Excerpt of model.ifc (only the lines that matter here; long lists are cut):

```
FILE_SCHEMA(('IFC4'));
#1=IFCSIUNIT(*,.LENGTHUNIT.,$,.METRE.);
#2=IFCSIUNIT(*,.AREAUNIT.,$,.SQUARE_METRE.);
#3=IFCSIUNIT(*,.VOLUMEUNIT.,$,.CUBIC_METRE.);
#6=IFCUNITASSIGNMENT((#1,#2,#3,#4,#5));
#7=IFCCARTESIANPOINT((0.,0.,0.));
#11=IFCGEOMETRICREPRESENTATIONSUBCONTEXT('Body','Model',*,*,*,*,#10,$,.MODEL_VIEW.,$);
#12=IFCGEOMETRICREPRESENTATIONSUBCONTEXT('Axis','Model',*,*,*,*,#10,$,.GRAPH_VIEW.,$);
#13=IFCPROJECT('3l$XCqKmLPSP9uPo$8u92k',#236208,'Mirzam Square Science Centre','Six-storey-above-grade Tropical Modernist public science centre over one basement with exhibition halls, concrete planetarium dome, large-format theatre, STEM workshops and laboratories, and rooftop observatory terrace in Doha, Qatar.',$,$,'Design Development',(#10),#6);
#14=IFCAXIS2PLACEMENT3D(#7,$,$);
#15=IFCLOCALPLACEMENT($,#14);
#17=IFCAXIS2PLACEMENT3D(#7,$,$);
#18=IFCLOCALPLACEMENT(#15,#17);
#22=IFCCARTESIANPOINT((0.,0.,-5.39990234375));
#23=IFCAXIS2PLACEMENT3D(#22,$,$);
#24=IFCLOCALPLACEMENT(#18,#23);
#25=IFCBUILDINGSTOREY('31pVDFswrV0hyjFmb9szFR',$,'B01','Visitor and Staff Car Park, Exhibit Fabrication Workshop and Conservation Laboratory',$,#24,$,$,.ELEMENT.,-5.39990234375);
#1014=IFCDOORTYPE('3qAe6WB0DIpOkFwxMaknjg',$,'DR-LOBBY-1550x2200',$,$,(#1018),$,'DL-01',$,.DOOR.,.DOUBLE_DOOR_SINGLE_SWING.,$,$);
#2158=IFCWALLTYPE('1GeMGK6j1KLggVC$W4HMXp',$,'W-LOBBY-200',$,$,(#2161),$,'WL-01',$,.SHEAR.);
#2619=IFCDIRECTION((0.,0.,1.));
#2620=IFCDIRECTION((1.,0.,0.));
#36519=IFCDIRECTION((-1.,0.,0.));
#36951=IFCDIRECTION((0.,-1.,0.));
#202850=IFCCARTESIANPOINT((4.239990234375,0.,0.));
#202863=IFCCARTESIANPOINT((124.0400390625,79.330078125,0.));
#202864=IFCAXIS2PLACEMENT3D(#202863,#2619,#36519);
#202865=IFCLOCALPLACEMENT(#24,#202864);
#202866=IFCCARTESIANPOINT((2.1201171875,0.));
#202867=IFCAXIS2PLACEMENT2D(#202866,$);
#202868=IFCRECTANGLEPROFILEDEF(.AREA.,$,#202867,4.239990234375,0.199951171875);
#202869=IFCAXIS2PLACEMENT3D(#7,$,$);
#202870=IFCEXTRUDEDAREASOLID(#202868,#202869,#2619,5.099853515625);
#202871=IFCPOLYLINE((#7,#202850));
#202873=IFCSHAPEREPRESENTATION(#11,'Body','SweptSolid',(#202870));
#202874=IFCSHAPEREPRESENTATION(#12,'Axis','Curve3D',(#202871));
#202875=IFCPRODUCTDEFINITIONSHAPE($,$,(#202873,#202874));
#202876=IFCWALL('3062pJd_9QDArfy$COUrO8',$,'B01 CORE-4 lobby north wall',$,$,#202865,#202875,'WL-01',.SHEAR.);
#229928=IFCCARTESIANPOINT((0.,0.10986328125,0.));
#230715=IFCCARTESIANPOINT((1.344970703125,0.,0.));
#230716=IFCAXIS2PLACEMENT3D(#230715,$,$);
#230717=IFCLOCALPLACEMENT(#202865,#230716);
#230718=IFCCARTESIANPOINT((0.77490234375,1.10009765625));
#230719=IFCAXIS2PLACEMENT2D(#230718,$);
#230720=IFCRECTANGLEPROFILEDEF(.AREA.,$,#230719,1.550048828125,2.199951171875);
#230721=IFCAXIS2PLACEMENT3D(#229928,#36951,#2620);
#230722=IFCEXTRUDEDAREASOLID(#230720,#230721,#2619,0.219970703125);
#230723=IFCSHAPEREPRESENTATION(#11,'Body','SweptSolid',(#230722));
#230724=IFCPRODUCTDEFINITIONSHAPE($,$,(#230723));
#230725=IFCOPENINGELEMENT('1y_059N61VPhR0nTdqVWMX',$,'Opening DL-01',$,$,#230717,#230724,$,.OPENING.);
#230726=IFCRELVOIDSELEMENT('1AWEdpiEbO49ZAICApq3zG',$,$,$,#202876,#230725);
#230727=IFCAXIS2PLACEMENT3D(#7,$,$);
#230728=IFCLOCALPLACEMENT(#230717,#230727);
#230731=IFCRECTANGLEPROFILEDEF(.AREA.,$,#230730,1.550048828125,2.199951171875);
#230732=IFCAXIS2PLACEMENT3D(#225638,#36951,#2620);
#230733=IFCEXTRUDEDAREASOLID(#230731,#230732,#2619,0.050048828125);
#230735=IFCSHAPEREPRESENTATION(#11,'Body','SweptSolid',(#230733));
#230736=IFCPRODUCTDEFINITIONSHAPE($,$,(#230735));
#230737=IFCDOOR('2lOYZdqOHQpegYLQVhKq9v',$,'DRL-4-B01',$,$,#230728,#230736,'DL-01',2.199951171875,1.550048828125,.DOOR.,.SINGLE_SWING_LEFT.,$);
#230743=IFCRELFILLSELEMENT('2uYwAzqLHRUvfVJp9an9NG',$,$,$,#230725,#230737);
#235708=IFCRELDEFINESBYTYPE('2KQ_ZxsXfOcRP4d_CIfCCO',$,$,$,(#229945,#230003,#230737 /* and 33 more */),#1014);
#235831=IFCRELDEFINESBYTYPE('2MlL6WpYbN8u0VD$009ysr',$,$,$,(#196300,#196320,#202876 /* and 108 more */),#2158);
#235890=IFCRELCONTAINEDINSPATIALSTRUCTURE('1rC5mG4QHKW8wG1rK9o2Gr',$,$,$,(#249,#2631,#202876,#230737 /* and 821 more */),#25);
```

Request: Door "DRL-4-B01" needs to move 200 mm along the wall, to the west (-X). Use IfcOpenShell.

```python
import ifcopenshell
import ifcopenshell.api.geometry
import ifcopenshell.util.placement
import ifcopenshell.util.unit

model = ifcopenshell.open("model.ifc")
unit_scale = ifcopenshell.util.unit.calculate_unit_scale(model)

door = model.by_id(230737)
opening = door.FillsVoids[0].RelatingOpeningElement
wall = opening.VoidsElements[0].RelatingBuildingElement

wall_matrix = ifcopenshell.util.placement.get_local_placement(wall.ObjectPlacement)
shift = wall_matrix[:3, 0] * 0.2 / unit_scale
before = ifcopenshell.util.placement.get_local_placement(door.ObjectPlacement)[:3, 3].copy()

# The door is placed relative to its opening, so it follows when the opening moves.
matrix = ifcopenshell.util.placement.get_local_placement(opening.ObjectPlacement)
matrix[:3, 3] += shift
ifcopenshell.api.geometry.edit_object_placement(
    model, product=opening, matrix=matrix, is_si=False, should_transform_children=True
)

after = ifcopenshell.util.placement.get_local_placement(door.ObjectPlacement)[:3, 3]
print("door moved by", (after - before).round(3) + 0.0)

model.write("model_updated.ifc")
```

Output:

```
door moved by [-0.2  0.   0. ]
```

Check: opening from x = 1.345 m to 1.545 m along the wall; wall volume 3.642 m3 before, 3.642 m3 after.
